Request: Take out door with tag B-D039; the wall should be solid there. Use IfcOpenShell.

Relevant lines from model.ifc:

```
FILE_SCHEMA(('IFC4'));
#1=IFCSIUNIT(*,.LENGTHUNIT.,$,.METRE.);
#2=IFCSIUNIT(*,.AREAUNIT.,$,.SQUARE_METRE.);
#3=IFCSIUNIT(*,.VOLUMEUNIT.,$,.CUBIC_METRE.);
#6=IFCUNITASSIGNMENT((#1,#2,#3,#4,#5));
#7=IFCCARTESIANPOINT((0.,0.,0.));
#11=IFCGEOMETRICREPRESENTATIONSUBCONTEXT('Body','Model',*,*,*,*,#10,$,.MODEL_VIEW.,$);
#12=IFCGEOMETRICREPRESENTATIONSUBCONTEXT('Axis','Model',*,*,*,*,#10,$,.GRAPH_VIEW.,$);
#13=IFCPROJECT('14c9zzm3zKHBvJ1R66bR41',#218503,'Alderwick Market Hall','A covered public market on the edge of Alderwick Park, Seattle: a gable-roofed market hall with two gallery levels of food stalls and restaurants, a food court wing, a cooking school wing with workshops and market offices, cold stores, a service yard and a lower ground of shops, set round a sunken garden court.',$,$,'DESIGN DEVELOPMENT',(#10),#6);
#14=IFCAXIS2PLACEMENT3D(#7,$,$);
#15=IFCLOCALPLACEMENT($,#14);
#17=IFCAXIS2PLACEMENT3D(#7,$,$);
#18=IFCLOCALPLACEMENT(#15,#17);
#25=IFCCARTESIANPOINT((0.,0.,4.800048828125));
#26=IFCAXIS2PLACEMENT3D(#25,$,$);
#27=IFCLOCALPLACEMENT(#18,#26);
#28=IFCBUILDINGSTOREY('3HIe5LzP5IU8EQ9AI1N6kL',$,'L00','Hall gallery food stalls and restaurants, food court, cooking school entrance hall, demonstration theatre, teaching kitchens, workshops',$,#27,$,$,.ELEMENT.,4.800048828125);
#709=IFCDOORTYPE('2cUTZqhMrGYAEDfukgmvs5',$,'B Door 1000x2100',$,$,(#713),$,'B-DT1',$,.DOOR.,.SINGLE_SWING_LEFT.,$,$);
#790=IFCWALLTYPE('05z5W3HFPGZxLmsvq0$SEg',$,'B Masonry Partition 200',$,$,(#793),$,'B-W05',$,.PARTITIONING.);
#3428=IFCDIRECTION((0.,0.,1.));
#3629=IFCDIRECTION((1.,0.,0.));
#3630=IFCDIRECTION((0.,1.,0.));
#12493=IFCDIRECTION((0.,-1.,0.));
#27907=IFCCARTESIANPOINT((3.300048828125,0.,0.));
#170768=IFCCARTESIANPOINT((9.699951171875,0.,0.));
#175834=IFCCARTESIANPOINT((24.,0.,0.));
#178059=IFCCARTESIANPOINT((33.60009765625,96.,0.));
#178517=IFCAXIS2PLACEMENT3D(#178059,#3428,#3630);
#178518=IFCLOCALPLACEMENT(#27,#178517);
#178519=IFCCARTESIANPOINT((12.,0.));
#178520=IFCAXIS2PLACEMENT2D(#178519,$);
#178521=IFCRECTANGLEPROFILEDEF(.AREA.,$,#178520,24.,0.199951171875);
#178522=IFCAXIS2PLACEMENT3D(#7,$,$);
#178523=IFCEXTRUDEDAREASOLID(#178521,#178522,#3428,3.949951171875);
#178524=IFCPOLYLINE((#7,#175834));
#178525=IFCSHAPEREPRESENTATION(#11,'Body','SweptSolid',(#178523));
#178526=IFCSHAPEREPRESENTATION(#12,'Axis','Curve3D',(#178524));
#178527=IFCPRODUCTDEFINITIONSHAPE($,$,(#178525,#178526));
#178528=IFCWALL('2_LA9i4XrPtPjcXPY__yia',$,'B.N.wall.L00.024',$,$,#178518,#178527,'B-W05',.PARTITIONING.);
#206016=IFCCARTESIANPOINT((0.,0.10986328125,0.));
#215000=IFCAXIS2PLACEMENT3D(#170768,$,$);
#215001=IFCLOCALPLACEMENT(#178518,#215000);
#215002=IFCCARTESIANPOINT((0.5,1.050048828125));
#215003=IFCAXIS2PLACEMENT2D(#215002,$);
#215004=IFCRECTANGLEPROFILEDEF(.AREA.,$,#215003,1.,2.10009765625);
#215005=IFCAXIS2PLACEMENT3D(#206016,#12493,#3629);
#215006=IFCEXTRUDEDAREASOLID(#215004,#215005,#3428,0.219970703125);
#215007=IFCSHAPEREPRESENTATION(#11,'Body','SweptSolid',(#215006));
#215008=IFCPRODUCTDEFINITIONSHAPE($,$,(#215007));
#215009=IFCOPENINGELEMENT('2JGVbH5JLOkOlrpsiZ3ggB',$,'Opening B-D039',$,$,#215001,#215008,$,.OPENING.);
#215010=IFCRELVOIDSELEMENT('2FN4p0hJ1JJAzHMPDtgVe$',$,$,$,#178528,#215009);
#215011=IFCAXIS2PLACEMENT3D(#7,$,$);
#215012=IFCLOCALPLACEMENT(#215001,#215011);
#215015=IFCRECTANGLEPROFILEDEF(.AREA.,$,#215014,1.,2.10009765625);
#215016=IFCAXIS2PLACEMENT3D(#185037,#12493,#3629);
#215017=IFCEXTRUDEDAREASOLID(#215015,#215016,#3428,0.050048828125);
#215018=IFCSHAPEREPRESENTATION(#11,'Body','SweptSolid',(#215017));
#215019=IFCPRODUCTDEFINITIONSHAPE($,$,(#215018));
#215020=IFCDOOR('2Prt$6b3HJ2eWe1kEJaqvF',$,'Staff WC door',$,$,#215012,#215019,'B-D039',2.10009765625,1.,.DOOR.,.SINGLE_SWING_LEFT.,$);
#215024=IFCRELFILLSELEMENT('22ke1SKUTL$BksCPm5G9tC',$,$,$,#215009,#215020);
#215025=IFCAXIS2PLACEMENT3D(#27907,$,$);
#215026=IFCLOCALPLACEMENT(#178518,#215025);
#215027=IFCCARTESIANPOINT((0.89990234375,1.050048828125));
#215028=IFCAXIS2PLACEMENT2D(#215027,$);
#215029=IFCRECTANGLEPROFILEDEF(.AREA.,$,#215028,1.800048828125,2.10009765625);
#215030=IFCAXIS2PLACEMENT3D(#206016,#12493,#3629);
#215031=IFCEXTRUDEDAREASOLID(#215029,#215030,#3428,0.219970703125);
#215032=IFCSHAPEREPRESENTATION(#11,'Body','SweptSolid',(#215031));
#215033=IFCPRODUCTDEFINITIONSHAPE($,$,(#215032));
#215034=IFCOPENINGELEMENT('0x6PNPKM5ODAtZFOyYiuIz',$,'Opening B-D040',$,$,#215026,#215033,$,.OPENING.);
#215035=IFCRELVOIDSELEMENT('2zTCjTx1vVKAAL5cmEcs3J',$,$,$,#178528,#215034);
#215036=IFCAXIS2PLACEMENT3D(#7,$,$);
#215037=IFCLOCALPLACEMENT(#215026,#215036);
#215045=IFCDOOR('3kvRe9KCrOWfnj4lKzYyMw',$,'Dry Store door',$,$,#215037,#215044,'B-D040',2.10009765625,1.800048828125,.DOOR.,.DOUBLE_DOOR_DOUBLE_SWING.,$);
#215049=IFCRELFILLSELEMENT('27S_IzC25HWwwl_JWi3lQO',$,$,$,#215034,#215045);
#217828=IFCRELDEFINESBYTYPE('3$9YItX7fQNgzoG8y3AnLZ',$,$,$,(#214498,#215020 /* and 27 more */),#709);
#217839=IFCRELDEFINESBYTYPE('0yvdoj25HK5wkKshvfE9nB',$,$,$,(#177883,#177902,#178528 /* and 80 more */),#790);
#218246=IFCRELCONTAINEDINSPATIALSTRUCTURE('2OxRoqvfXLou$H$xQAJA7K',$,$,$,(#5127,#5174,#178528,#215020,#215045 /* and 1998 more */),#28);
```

```python
import ifcopenshell
import ifcopenshell.api.feature
import ifcopenshell.api.root
import ifcopenshell.geom
import ifcopenshell.util.shape

model = ifcopenshell.open("model.ifc")
settings = ifcopenshell.geom.settings()


def volume(element):
    """Net volume in cubic metres, openings subtracted."""
    shape = ifcopenshell.geom.create_shape(settings, element)
    return ifcopenshell.util.shape.get_volume(shape.geometry)


door = model.by_id(215020)
opening = door.FillsVoids[0].RelatingOpeningElement
wall = opening.VoidsElements[0].RelatingBuildingElement
before = volume(wall)

ifcopenshell.api.root.remove_product(model, product=door)
ifcopenshell.api.feature.remove_feature(model, feature=opening)

after = volume(wall)

print(f"wall volume {before:.3f} -> {after:.3f} m3")

model.write("model_rev.ifc")
```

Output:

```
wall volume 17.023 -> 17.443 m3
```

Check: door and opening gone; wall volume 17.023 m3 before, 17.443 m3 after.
